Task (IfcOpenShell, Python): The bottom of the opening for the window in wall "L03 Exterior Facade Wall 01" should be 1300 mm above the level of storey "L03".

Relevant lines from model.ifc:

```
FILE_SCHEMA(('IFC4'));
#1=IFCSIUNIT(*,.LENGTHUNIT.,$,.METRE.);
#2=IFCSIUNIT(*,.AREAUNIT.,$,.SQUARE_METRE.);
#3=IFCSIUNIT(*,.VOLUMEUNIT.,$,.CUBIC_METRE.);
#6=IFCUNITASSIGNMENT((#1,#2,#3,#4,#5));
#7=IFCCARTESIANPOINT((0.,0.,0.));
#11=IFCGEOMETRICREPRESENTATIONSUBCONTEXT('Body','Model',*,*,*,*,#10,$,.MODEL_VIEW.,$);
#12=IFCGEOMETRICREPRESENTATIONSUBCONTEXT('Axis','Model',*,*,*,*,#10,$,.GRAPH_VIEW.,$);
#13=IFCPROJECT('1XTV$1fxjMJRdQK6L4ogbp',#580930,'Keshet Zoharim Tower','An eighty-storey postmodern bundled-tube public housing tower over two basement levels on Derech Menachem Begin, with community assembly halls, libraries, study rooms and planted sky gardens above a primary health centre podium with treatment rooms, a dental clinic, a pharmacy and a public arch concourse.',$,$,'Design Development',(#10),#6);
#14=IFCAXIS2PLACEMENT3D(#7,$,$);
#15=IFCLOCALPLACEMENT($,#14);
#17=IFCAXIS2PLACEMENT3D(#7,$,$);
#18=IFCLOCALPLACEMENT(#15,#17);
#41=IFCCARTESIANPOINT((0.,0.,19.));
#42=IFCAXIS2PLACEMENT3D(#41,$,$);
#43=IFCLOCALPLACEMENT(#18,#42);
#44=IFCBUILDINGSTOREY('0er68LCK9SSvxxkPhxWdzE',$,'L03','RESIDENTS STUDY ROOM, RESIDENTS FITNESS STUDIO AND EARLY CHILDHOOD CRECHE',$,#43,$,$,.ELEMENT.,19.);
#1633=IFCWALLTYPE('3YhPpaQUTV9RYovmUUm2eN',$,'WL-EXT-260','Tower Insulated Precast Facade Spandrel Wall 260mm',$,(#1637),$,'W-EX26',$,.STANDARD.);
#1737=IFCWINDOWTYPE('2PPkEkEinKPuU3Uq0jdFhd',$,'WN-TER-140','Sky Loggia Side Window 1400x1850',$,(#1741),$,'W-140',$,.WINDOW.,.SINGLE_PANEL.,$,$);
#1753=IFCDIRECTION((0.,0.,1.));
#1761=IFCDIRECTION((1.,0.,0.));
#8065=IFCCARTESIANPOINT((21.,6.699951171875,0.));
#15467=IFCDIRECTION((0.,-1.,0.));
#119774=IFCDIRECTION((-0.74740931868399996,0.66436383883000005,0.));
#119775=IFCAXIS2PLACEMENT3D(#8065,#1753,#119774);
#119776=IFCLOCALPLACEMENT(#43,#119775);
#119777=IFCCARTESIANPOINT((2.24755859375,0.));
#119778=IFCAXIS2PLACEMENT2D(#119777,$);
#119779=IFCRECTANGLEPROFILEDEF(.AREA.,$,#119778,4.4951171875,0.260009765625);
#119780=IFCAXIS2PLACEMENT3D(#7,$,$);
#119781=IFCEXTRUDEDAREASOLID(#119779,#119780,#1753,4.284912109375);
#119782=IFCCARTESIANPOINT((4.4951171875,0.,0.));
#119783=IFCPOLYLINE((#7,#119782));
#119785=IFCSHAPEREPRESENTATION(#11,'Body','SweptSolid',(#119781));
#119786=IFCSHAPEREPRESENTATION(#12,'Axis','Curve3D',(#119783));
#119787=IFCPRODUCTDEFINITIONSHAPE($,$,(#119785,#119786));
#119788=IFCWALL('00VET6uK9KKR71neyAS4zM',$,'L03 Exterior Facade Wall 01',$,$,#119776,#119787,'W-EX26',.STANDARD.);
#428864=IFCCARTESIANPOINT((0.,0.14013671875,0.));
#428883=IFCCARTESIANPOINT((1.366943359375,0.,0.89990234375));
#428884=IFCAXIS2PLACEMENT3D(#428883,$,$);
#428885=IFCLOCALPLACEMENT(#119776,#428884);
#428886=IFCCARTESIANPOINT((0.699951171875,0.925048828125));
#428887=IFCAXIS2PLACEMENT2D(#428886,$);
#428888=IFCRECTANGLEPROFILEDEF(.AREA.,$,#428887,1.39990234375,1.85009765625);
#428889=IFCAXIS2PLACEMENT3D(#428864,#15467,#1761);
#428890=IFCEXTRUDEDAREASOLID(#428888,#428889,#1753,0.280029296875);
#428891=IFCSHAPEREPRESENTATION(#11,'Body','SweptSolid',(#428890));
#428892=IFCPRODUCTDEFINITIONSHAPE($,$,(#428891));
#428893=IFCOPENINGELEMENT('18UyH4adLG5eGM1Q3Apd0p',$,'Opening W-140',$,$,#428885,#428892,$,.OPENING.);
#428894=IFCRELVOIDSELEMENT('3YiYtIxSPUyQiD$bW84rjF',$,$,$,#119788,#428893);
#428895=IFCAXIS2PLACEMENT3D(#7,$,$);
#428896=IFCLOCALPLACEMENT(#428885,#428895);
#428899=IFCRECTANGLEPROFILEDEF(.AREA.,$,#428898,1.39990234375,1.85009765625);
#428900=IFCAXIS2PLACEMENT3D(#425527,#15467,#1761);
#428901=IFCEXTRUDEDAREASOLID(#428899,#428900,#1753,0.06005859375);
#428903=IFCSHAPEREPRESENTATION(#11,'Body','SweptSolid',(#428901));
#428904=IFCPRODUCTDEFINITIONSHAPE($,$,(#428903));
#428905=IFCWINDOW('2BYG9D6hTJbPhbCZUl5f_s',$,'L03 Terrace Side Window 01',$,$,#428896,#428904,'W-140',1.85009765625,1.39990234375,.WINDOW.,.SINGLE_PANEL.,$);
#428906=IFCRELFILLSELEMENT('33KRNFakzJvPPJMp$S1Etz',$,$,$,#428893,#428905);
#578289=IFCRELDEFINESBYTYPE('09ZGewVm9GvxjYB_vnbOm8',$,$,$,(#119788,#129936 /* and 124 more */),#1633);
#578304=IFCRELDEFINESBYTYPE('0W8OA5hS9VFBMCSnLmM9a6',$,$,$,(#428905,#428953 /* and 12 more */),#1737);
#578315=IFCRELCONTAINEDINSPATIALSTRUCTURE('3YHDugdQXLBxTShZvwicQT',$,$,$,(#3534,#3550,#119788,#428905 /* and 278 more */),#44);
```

```python
import numpy as np
import ifcopenshell
import ifcopenshell.api.geometry
import ifcopenshell.geom
import ifcopenshell.util.element
import ifcopenshell.util.placement
import ifcopenshell.util.shape
import ifcopenshell.util.unit

model = ifcopenshell.open("model.ifc")
unit_scale = ifcopenshell.util.unit.calculate_unit_scale(model)

window = model.by_guid("2BYG9D6hTJbPhbCZUl5f_s")
opening = window.FillsVoids[0].RelatingOpeningElement
storey = ifcopenshell.util.element.get_container(window, ifc_class="IfcBuildingStorey")
level = ifcopenshell.util.placement.get_local_placement(storey.ObjectPlacement)[2, 3]

# The opening's origin need not be at the sill, so measure its lowest point.
shape = ifcopenshell.geom.create_shape(ifcopenshell.geom.settings(), opening)
bottom = ifcopenshell.util.shape.get_shape_bottom_elevation(shape, shape.geometry) / unit_scale
dz = level + 1.3 - bottom

shift = np.array([0.0, 0.0, dz])
# The window is placed relative to its opening, so it follows when the opening moves.
matrix = ifcopenshell.util.placement.get_local_placement(opening.ObjectPlacement)
matrix[:3, 3] += shift
ifcopenshell.api.geometry.edit_object_placement(
    model, product=opening, matrix=matrix, is_si=False, should_transform_children=True
)

print(f"moved by {dz * unit_scale:+.3f} m")

model.write("model_edited.ifc")
```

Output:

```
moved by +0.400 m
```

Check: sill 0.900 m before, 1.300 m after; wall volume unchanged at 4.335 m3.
